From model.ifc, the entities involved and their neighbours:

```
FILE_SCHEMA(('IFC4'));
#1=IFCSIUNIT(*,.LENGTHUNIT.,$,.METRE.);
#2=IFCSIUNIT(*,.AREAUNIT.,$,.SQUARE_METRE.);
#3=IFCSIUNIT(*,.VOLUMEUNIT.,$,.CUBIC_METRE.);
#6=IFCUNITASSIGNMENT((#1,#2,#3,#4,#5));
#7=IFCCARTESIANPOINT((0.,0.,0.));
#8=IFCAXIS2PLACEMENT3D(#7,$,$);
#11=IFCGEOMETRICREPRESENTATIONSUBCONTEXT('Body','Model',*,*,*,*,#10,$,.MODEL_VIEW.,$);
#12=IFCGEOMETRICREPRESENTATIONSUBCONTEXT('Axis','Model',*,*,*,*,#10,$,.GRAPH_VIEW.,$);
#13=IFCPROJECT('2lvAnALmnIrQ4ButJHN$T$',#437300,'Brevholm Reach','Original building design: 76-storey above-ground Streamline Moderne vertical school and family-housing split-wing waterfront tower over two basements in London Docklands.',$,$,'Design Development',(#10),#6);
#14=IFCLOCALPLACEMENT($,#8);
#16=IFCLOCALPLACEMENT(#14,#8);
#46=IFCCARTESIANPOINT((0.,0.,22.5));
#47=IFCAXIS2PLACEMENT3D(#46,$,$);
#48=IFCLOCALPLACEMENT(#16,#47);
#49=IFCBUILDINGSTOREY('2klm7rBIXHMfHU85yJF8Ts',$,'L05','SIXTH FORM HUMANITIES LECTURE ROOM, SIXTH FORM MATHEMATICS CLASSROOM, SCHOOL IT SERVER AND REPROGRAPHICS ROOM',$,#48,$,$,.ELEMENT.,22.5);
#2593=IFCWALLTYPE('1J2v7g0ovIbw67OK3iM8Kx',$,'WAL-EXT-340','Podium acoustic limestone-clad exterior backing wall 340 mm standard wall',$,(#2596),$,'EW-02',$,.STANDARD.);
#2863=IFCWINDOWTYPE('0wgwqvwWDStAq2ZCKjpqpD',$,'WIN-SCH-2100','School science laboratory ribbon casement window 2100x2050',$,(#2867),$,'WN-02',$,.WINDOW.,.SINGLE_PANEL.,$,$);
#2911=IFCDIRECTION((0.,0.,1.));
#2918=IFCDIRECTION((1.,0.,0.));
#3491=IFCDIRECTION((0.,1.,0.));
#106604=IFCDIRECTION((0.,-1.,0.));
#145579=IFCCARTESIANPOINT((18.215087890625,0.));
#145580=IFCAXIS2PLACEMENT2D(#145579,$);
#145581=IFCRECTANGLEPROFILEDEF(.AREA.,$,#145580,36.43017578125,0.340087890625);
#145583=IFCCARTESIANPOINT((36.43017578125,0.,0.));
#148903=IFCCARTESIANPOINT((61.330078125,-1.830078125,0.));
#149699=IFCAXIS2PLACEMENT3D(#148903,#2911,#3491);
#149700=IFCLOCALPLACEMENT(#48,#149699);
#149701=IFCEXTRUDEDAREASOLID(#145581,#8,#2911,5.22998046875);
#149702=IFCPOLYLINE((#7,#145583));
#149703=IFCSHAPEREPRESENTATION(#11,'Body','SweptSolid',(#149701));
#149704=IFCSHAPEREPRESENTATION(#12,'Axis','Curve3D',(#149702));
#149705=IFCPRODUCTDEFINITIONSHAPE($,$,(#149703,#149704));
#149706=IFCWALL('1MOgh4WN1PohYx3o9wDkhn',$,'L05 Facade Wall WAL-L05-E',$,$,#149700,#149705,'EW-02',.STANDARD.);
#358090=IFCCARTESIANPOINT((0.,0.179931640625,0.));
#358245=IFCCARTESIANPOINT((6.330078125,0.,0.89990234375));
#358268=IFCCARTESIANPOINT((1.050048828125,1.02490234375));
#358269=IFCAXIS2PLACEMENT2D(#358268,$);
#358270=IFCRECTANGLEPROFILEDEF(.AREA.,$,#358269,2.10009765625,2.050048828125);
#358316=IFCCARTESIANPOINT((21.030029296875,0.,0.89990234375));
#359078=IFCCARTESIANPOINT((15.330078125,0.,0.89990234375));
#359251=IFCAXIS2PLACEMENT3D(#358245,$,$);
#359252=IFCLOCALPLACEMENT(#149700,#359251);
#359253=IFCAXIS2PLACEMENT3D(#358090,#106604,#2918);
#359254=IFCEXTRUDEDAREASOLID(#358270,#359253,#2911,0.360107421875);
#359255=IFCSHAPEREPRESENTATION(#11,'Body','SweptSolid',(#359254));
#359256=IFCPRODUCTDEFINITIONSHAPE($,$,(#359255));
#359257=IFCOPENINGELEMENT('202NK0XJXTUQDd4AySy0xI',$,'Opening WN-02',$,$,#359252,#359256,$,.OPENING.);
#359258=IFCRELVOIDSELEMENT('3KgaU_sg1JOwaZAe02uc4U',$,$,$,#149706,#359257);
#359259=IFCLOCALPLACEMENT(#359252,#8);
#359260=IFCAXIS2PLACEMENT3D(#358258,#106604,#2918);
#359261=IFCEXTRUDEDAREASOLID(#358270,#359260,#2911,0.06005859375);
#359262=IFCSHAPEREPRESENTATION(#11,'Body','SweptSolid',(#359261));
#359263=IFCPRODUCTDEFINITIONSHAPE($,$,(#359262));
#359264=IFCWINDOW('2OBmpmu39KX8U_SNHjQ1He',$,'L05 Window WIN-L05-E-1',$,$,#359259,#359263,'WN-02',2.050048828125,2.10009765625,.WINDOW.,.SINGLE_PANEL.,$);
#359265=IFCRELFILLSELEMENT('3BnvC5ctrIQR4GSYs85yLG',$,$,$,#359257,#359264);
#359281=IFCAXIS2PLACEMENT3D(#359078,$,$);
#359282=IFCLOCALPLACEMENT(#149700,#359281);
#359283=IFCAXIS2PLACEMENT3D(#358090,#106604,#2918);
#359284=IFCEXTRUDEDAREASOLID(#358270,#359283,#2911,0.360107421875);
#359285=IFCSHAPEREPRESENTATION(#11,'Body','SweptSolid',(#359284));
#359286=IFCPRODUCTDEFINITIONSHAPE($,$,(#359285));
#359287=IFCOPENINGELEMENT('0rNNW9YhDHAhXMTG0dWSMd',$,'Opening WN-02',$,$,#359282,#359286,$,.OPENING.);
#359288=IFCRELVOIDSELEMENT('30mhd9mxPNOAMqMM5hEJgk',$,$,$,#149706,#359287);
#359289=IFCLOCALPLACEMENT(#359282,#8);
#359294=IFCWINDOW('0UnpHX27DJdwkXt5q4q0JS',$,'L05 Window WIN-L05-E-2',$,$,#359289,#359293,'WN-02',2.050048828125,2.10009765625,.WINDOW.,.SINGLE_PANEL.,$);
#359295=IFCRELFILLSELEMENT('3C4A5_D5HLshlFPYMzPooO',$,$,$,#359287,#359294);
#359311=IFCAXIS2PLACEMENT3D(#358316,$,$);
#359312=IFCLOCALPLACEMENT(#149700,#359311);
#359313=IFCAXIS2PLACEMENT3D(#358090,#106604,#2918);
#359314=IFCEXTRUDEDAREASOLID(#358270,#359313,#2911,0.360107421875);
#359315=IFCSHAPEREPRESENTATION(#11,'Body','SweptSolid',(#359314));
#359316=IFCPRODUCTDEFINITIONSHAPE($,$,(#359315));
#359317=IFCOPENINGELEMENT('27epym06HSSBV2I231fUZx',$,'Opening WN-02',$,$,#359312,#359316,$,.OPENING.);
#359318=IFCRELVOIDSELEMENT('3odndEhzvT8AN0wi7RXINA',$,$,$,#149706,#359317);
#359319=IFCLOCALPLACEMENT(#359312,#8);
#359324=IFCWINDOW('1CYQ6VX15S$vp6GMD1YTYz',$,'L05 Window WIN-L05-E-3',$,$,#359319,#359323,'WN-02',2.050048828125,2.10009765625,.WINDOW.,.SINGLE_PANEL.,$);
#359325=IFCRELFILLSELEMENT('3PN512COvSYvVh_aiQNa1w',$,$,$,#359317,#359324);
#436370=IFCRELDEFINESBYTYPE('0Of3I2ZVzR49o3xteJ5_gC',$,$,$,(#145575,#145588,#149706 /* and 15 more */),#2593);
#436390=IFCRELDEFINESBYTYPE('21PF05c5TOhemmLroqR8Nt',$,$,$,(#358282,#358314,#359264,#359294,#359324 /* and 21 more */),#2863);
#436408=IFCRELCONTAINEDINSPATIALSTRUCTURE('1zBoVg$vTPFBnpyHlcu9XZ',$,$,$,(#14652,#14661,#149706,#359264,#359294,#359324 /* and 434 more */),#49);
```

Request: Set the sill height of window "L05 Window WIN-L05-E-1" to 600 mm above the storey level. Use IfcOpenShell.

```python
import numpy as np
import ifcopenshell
import ifcopenshell.api.geometry
import ifcopenshell.geom
import ifcopenshell.util.element
import ifcopenshell.util.placement
import ifcopenshell.util.shape
import ifcopenshell.util.unit

model = ifcopenshell.open("model.ifc")
unit_scale = ifcopenshell.util.unit.calculate_unit_scale(model)

window = model.by_guid("2OBmpmu39KX8U_SNHjQ1He")
opening = window.FillsVoids[0].RelatingOpeningElement
storey = ifcopenshell.util.element.get_container(window, ifc_class="IfcBuildingStorey")
level = ifcopenshell.util.placement.get_local_placement(storey.ObjectPlacement)[2, 3]

# The opening's origin need not be at the sill, so measure its lowest point.
shape = ifcopenshell.geom.create_shape(ifcopenshell.geom.settings(), opening)
bottom = ifcopenshell.util.shape.get_shape_bottom_elevation(shape, shape.geometry) / unit_scale
dz = level + 0.6 / unit_scale - bottom

shift = np.array([0.0, 0.0, dz])
# The window is placed relative to its opening, so it follows when the opening moves.
matrix = ifcopenshell.util.placement.get_local_placement(opening.ObjectPlacement)
matrix[:3, 3] += shift
ifcopenshell.api.geometry.edit_object_placement(
    model, product=opening, matrix=matrix, is_si=False, should_transform_children=True
)

print(f"moved by {dz * unit_scale:+.3f} m")

model.write("model_edited.ifc")
```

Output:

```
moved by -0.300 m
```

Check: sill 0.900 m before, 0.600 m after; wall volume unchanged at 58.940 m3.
